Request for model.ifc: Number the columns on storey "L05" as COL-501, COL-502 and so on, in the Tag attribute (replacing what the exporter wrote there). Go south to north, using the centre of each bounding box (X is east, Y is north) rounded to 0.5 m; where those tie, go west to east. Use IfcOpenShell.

First a look at what the model holds.

```python
import ifcopenshell
import ifcopenshell.util.element
import ifcopenshell.util.placement

model = ifcopenshell.open("model.ifc")
print(model.schema)
storey = next(s for s in model.by_type("IfcBuildingStorey") if s.Name == "L05")
columns = [e for e in ifcopenshell.util.element.get_decomposition(storey) if e.is_a("IfcColumn")]
for e in sorted(columns, key=lambda e: e.id()):
    origin = ifcopenshell.util.placement.get_local_placement(e.ObjectPlacement)[:3, 3]
    print(e.id(), e.Tag, e.Name, origin.round(2) + 0.0, sep=" | ")
```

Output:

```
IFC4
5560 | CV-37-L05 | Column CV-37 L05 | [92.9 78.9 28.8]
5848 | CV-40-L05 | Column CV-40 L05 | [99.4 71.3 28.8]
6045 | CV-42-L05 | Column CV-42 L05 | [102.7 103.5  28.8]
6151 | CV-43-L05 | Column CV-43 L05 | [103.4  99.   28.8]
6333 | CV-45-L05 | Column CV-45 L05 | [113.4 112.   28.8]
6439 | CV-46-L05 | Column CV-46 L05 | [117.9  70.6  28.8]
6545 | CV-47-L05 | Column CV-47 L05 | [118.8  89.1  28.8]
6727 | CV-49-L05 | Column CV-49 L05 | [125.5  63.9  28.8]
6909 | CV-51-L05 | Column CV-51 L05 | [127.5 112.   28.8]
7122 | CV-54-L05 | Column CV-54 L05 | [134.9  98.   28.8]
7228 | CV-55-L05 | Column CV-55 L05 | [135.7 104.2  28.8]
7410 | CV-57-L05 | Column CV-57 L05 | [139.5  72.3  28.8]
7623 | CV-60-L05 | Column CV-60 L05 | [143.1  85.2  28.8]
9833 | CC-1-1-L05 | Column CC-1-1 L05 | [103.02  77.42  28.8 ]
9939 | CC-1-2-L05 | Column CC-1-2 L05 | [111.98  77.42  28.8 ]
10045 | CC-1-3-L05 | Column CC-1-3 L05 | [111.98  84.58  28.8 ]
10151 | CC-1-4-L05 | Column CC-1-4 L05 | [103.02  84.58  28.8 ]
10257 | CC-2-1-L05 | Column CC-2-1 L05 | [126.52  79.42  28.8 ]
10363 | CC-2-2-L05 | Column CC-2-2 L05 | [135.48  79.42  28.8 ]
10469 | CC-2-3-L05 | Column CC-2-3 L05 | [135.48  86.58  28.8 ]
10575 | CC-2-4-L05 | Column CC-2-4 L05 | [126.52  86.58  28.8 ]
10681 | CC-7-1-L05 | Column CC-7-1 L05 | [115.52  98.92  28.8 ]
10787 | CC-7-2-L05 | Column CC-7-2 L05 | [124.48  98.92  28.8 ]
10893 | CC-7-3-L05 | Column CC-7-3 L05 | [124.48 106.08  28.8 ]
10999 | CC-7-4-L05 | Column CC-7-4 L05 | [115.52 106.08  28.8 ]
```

```python
import ifcopenshell
import ifcopenshell.geom
import ifcopenshell.util.element
import ifcopenshell.util.shape

model = ifcopenshell.open("model.ifc")
settings = ifcopenshell.geom.settings()
settings.set("use-world-coords", True)


def centre(element):
    shape = ifcopenshell.geom.create_shape(settings, element)
    return ifcopenshell.util.shape.get_bbox_centroid(shape.geometry)


storey = next(s for s in model.by_type("IfcBuildingStorey") if s.Name == "L05")
columns = [e for e in ifcopenshell.util.element.get_decomposition(storey) if e.is_a("IfcColumn")]

# Insertion points can sit at a corner or the storey origin, so sort by the geometry (in metres).
centres = {e: centre(e) for e in columns}
columns.sort(key=lambda e: (round(centres[e][1] / 0.5), centres[e][0]))

for i, e in enumerate(columns, start=1):
    number = f"COL-5{i:02d}"
    e.Tag = number
    print(e.id(), number)

model.write("model_v2.ifc")
```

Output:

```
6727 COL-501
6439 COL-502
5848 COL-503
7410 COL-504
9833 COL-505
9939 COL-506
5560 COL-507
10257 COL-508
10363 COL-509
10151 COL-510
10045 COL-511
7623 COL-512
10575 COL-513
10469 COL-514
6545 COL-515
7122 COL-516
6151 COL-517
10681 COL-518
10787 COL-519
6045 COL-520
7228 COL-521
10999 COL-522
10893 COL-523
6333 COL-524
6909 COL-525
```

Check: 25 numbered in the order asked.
